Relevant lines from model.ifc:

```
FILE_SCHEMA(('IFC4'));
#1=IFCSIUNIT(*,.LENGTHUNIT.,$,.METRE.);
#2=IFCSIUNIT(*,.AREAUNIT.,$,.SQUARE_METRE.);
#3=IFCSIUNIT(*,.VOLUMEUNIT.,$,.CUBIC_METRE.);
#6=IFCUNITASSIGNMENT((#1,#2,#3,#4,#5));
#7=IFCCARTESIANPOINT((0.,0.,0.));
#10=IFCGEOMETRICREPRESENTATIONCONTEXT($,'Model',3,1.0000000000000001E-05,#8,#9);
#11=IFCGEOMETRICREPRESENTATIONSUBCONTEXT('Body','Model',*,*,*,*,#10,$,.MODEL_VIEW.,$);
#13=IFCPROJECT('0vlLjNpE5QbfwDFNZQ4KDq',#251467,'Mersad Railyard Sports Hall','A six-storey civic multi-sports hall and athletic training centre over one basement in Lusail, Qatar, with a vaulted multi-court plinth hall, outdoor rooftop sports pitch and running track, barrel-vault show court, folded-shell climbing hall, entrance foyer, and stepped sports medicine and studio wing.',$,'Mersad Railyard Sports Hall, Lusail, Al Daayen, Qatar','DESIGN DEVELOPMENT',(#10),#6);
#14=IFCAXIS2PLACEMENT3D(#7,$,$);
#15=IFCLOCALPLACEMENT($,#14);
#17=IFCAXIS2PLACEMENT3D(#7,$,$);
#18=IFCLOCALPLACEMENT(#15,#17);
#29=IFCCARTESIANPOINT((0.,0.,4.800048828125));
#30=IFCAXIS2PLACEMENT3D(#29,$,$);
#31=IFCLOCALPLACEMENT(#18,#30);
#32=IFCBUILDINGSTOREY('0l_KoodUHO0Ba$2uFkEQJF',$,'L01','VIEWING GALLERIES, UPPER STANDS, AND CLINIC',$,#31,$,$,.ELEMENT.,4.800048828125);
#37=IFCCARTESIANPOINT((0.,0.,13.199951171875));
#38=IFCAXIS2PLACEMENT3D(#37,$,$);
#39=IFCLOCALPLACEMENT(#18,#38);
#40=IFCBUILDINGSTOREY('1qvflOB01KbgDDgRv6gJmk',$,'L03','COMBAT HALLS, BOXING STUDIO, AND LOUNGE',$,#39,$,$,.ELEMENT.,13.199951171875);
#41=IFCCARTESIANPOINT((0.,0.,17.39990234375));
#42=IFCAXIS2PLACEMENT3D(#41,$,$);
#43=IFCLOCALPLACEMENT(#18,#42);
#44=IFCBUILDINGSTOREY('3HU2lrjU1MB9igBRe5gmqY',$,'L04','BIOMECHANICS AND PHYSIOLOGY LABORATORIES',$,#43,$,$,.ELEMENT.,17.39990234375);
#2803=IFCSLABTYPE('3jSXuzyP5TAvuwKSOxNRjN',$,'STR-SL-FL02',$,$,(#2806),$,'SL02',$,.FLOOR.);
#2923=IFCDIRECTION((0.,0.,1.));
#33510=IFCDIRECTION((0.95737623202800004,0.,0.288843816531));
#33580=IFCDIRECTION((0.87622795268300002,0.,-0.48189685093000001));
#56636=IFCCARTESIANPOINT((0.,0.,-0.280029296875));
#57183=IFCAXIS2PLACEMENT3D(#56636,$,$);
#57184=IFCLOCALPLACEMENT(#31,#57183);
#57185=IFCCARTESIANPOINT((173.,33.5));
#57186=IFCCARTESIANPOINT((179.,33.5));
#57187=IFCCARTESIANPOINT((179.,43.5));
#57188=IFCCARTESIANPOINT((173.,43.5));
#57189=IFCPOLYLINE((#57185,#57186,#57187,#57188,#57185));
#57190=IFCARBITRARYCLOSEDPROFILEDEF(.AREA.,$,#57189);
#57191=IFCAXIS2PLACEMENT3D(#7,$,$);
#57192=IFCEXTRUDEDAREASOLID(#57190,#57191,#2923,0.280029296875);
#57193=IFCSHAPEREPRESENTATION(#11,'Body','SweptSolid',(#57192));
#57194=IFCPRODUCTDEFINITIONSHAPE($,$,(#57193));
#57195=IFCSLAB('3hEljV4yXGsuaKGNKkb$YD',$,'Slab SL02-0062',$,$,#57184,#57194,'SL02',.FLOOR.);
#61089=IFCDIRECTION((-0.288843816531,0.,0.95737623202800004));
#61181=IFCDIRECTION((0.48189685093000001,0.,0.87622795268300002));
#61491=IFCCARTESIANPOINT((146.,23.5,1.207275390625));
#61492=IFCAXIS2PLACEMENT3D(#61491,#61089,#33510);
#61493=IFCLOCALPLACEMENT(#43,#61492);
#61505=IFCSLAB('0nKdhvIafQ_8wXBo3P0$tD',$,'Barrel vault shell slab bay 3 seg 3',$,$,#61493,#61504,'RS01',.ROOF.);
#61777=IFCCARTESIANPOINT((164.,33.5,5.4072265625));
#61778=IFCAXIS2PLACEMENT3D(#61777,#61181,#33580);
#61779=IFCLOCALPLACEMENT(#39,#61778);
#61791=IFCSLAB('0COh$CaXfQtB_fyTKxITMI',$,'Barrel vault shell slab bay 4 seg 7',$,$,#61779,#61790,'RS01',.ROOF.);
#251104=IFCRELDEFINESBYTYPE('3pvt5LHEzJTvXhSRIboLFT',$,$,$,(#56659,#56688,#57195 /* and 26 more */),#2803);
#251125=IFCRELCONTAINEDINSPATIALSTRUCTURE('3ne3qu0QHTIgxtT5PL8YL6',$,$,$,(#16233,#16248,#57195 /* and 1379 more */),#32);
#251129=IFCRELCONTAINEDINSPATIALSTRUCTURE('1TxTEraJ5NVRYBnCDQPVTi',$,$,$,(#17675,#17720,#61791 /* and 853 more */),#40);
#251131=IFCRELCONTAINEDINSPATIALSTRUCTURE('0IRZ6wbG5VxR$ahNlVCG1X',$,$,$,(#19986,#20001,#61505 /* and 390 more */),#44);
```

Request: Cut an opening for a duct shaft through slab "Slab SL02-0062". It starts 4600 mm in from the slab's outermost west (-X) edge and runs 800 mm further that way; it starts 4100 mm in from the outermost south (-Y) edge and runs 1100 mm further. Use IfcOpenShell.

```python
import numpy as np
import ifcopenshell
import ifcopenshell.api.feature
import ifcopenshell.api.geometry
import ifcopenshell.api.root
import ifcopenshell.geom
import ifcopenshell.util.placement
import ifcopenshell.util.representation
import ifcopenshell.util.shape
import ifcopenshell.util.unit

model = ifcopenshell.open("model.ifc")
unit_scale = ifcopenshell.util.unit.calculate_unit_scale(model)
settings = ifcopenshell.geom.settings()


def volume(element):
    """Net volume in cubic metres, openings subtracted."""
    shape = ifcopenshell.geom.create_shape(settings, element)
    return ifcopenshell.util.shape.get_volume(shape.geometry)


slab = model.by_guid("3hEljV4yXGsuaKGNKkb$YD")
before = volume(slab)

# Extent in the slab's own axes, in metres. The edges named are its -X and -Y sides.
slab_shape = ifcopenshell.geom.create_shape(settings, slab)
vertices = ifcopenshell.util.shape.get_vertices(slab_shape.geometry)
x_min, y_min, bottom = vertices.min(axis=0)
top = vertices[:, 2].max()

opening = ifcopenshell.api.root.create_entity(model, ifc_class="IfcOpeningElement", name="Duct shaft opening", predefined_type="OPENING")
context = ifcopenshell.util.representation.get_context(model, "Model", "Body", "MODEL_VIEW")
width, depth = 0.8, 1.1
outline = [(0.0, 0.0), (width, 0.0), (width, depth), (0.0, depth), (0.0, 0.0)]
# Overshoot both faces by 50 mm so the cut is clean.
shape = ifcopenshell.api.geometry.add_slab_representation(
    model, context=context, depth=top - bottom + 0.1, polyline=outline
)
ifcopenshell.api.geometry.assign_representation(model, product=opening, representation=shape)

matrix = ifcopenshell.util.placement.get_local_placement(slab.ObjectPlacement)
matrix[:, 3] = matrix @ np.append(np.array([x_min + 4.6, y_min + 4.1, bottom - 0.05]) / unit_scale, 1.0)
ifcopenshell.api.geometry.edit_object_placement(model, product=opening, matrix=matrix, is_si=False)
ifcopenshell.api.feature.add_feature(model, feature=opening, element=slab)

after = volume(slab)

print(f"slab volume {before:.3f} -> {after:.3f} m3")

model.write("model-out.ifc")
```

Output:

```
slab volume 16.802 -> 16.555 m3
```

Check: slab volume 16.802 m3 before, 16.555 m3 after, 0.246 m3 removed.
